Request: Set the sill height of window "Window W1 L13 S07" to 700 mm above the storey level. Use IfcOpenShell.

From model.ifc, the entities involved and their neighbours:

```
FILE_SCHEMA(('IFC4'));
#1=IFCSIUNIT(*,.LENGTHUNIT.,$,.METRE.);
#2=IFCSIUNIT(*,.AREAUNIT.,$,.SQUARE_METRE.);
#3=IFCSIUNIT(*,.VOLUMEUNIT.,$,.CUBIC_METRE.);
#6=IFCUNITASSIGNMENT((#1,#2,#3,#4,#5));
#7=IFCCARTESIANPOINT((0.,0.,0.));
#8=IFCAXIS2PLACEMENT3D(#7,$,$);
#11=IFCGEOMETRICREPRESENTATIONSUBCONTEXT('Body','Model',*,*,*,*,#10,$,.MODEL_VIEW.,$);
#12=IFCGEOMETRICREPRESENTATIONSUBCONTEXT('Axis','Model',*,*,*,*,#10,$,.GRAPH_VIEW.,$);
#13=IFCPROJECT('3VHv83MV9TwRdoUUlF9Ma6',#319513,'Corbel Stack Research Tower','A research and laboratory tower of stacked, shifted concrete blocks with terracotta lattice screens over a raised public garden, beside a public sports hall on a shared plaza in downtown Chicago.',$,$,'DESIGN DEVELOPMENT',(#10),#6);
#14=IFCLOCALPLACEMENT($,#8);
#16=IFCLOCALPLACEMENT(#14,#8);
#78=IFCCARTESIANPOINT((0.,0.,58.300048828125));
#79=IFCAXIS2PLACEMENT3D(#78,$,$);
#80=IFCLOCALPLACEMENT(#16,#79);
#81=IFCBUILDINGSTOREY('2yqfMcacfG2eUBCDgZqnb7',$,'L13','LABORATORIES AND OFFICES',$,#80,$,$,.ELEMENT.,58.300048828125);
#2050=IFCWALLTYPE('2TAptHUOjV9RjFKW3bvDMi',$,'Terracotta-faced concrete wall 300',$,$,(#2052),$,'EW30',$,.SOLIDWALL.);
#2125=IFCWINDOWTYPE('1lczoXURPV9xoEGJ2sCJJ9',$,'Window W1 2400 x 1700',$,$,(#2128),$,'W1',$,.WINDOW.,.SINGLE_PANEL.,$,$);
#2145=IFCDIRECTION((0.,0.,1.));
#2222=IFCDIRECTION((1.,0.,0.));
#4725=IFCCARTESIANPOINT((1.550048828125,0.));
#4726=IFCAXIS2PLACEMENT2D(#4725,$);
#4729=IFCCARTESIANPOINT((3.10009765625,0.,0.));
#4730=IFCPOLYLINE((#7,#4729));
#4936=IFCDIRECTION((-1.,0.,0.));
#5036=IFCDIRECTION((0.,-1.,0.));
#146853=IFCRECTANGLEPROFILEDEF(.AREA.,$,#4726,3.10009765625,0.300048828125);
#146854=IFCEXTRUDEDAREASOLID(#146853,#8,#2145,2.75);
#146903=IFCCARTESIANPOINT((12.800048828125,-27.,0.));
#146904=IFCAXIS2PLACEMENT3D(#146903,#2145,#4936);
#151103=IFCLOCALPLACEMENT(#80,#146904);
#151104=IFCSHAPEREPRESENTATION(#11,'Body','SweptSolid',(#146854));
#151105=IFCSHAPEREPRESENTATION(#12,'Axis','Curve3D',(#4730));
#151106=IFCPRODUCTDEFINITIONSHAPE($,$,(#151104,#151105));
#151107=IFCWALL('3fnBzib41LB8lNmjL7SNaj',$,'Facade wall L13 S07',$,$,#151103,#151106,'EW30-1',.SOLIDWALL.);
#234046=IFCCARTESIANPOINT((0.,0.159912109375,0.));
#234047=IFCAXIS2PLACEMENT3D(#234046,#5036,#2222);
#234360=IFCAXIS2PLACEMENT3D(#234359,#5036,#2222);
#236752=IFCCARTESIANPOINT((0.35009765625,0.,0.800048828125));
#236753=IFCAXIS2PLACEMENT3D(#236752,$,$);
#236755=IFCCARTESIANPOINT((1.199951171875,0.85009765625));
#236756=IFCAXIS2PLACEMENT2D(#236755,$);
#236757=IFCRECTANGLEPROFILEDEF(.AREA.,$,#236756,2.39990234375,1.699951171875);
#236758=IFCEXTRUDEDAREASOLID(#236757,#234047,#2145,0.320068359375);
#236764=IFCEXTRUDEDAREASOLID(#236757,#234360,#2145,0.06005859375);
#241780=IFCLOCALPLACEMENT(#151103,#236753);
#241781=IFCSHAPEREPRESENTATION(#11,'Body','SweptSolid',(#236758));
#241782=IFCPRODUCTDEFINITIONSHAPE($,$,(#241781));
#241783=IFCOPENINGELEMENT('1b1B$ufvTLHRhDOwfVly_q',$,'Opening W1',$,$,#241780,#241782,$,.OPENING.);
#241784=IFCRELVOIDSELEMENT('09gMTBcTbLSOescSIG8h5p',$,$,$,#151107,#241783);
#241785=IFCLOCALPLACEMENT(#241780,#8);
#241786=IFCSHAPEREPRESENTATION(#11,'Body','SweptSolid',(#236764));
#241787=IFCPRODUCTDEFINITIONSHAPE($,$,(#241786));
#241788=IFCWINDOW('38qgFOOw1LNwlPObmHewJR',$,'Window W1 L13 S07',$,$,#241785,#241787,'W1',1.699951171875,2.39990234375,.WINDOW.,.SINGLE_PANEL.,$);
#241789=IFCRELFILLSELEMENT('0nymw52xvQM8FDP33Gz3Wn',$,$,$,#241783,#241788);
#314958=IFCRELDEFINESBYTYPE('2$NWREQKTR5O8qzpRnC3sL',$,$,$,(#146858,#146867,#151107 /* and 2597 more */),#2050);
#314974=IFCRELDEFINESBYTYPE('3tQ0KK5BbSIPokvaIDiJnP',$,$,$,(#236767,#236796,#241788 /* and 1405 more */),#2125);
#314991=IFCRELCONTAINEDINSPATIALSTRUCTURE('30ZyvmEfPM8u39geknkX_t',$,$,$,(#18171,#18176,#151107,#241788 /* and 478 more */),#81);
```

```python
import numpy as np
import ifcopenshell
import ifcopenshell.api.geometry
import ifcopenshell.geom
import ifcopenshell.util.element
import ifcopenshell.util.placement
import ifcopenshell.util.shape
import ifcopenshell.util.unit

model = ifcopenshell.open("model.ifc")
unit_scale = ifcopenshell.util.unit.calculate_unit_scale(model)

window = model.by_guid("38qgFOOw1LNwlPObmHewJR")
opening = window.FillsVoids[0].RelatingOpeningElement
storey = ifcopenshell.util.element.get_container(window, ifc_class="IfcBuildingStorey")
level = ifcopenshell.util.placement.get_local_placement(storey.ObjectPlacement)[2, 3]

# The opening's origin need not be at the sill, so measure its lowest point.
shape = ifcopenshell.geom.create_shape(ifcopenshell.geom.settings(), opening)
bottom = ifcopenshell.util.shape.get_shape_bottom_elevation(shape, shape.geometry) / unit_scale
dz = level + 0.7 / unit_scale - bottom

shift = np.array([0.0, 0.0, dz])
# The window is placed relative to its opening, so it follows when the opening moves.
matrix = ifcopenshell.util.placement.get_local_placement(opening.ObjectPlacement)
matrix[:3, 3] += shift
ifcopenshell.api.geometry.edit_object_placement(
    model, product=opening, matrix=matrix, is_si=False, should_transform_children=True
)

print(f"moved by {dz * unit_scale:+.3f} m")

model.write("model_edited.ifc")
```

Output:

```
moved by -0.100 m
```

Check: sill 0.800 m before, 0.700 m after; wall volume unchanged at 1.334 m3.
